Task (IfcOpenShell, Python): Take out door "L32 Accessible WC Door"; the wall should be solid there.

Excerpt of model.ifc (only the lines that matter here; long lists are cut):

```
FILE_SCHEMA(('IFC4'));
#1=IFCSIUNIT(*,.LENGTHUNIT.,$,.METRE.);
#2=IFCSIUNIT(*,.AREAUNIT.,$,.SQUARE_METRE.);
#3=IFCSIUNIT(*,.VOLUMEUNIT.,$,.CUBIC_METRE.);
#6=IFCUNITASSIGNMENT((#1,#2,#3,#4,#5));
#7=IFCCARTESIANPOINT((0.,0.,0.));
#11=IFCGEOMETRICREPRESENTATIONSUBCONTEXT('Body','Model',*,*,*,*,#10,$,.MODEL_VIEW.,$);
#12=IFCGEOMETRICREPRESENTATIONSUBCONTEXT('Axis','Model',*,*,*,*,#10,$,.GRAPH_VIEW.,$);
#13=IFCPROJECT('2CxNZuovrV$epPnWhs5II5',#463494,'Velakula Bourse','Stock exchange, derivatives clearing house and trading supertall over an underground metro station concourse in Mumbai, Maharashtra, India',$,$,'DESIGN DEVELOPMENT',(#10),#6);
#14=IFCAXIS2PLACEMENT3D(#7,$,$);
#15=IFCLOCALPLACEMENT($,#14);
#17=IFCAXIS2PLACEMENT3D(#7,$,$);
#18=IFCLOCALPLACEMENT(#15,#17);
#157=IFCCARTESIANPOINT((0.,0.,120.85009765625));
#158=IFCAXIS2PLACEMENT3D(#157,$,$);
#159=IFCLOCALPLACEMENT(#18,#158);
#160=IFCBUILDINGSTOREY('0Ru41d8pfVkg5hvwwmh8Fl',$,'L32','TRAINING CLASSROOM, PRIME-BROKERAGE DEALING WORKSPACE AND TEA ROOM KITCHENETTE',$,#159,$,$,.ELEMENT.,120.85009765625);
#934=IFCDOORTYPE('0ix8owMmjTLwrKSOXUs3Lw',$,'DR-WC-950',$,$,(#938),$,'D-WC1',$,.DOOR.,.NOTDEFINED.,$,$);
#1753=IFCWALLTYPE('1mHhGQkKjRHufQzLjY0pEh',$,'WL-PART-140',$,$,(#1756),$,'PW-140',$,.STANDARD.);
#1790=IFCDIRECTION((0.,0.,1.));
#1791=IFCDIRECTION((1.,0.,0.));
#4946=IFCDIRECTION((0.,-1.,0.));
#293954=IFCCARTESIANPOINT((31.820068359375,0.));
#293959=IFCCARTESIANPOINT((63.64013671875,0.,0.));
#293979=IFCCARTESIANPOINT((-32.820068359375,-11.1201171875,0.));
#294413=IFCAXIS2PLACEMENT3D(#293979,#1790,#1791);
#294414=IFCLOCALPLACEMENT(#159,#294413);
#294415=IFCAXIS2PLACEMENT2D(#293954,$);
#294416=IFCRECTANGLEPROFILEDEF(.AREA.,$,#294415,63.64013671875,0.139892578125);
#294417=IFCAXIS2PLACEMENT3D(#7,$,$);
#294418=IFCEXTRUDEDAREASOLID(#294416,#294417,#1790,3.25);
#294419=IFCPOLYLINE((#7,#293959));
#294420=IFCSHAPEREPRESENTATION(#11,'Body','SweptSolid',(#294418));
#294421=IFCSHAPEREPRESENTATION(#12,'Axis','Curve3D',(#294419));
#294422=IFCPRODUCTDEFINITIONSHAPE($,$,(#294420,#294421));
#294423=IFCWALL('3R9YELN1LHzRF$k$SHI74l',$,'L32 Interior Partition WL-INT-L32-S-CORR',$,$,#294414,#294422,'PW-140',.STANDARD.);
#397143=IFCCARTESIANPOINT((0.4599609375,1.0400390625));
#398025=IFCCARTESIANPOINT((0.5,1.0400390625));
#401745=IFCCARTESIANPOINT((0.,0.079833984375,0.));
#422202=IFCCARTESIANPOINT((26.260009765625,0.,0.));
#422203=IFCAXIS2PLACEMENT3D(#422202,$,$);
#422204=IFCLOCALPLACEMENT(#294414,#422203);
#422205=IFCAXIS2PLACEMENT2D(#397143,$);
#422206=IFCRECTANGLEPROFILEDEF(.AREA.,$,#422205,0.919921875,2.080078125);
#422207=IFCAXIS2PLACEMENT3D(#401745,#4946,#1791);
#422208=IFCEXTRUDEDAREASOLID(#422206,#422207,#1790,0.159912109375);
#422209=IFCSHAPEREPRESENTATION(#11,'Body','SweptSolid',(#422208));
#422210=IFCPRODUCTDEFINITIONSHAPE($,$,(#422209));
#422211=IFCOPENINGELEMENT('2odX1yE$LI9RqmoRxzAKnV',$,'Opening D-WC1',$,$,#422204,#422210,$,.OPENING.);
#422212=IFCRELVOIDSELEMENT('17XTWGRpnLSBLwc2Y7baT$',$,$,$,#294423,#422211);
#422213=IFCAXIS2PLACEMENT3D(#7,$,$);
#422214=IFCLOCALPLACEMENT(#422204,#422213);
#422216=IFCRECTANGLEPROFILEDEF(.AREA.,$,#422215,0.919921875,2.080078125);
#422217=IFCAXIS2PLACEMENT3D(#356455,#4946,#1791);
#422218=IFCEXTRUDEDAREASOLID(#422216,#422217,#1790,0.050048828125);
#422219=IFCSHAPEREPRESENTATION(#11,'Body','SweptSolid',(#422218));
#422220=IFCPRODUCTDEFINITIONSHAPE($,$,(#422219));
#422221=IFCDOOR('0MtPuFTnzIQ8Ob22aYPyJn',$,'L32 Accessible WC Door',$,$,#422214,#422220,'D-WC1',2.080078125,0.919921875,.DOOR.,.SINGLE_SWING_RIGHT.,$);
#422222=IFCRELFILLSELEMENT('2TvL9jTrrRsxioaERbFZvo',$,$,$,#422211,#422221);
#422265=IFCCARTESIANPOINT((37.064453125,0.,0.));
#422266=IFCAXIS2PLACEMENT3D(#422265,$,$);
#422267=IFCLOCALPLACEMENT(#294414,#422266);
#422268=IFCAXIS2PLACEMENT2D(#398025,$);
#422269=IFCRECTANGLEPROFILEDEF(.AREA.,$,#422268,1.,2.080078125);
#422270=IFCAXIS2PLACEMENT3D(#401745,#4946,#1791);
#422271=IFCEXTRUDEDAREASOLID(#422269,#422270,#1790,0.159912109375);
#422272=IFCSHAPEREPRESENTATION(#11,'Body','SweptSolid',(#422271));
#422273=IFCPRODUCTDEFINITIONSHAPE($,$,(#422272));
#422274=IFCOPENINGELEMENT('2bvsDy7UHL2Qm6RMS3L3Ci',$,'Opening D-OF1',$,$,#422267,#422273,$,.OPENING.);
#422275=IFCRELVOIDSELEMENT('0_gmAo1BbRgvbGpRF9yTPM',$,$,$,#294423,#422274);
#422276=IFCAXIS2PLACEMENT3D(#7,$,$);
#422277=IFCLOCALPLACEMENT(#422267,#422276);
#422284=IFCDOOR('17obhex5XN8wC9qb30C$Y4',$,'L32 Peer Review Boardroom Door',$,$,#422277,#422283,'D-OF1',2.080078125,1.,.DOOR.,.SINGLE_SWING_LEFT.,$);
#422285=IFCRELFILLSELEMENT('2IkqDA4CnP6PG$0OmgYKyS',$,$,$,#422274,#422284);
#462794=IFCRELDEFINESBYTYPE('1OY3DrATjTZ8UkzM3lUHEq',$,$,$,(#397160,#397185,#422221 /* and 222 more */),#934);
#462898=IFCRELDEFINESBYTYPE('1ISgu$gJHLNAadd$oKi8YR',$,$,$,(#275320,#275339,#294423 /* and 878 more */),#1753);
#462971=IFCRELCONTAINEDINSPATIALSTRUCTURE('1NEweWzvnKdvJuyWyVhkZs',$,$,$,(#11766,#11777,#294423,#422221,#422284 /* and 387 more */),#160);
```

```python
import ifcopenshell
import ifcopenshell.api.feature
import ifcopenshell.api.root
import ifcopenshell.geom
import ifcopenshell.util.shape

model = ifcopenshell.open("model.ifc")
settings = ifcopenshell.geom.settings()


def volume(element):
    """Net volume in cubic metres, openings subtracted."""
    shape = ifcopenshell.geom.create_shape(settings, element)
    return ifcopenshell.util.shape.get_volume(shape.geometry)


door = model.by_guid("0MtPuFTnzIQ8Ob22aYPyJn")
opening = door.FillsVoids[0].RelatingOpeningElement
wall = opening.VoidsElements[0].RelatingBuildingElement
before = volume(wall)

ifcopenshell.api.root.remove_product(model, product=door)
ifcopenshell.api.feature.remove_feature(model, feature=opening)

after = volume(wall)

print(f"wall volume {before:.3f} -> {after:.3f} m3")

model.write("model_rev.ifc")
```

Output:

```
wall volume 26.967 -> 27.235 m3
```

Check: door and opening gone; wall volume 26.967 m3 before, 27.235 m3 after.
